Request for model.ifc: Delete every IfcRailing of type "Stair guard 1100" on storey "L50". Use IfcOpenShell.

First a look at what the model holds.

```python
import ifcopenshell
import ifcopenshell.util.element

model = ifcopenshell.open("model.ifc")
print(model.schema)
storey = next(s for s in model.by_type("IfcBuildingStorey") if s.Name == "L50")
railings = [e for e in ifcopenshell.util.element.get_decomposition(storey) if e.is_a("IfcRailing")]
seen = {}
for e in railings:
    element_type = ifcopenshell.util.element.get_type(e)
    name = element_type.Name if element_type not in (None, e) else None
    seen[name] = seen.get(name, 0) + 1
for name, count in sorted(seen.items(), key=str):
    print(count, "x", name)
```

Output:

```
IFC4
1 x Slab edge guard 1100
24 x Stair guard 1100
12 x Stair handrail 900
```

```python
import ifcopenshell
import ifcopenshell.api.root
import ifcopenshell.util.element

model = ifcopenshell.open("model.ifc")

storey = next(s for s in model.by_type("IfcBuildingStorey") if s.Name == "L50")
railings = [e for e in ifcopenshell.util.element.get_decomposition(storey) if e.is_a("IfcRailing")]
targets = [e for e in railings if (t := ifcopenshell.util.element.get_type(e)) not in (None, e) and t.Name == "Stair guard 1100"]

for e in targets:
    ifcopenshell.api.root.remove_product(model, product=e)
print(len(targets), "removed")

model.write("model_edited.ifc")
```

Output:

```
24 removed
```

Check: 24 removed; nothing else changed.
